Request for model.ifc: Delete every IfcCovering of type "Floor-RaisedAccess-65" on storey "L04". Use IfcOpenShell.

First a look at what the model holds.

```python
import ifcopenshell
import ifcopenshell.util.element

model = ifcopenshell.open("model.ifc")
print(model.schema)
storey = next(s for s in model.by_type("IfcBuildingStorey") if s.Name == "L04")
coverings = [e for e in ifcopenshell.util.element.get_decomposition(storey) if e.is_a("IfcCovering")]
seen = {}
for e in coverings:
    element_type = ifcopenshell.util.element.get_type(e)
    name = element_type.Name if element_type not in (None, e) else None
    seen[name] = seen.get(name, 0) + 1
for name, count in sorted(seen.items(), key=str):
    print(count, "x", name)
```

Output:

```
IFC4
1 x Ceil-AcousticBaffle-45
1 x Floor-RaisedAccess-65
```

```python
import ifcopenshell
import ifcopenshell.api.root
import ifcopenshell.util.element

model = ifcopenshell.open("model.ifc")

storey = next(s for s in model.by_type("IfcBuildingStorey") if s.Name == "L04")
coverings = [e for e in ifcopenshell.util.element.get_decomposition(storey) if e.is_a("IfcCovering")]
targets = [e for e in coverings if (t := ifcopenshell.util.element.get_type(e)) not in (None, e) and t.Name == "Floor-RaisedAccess-65"]

for e in targets:
    ifcopenshell.api.root.remove_product(model, product=e)
print(len(targets), "removed")

model.write("model_edited.ifc")
```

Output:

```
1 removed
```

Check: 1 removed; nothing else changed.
